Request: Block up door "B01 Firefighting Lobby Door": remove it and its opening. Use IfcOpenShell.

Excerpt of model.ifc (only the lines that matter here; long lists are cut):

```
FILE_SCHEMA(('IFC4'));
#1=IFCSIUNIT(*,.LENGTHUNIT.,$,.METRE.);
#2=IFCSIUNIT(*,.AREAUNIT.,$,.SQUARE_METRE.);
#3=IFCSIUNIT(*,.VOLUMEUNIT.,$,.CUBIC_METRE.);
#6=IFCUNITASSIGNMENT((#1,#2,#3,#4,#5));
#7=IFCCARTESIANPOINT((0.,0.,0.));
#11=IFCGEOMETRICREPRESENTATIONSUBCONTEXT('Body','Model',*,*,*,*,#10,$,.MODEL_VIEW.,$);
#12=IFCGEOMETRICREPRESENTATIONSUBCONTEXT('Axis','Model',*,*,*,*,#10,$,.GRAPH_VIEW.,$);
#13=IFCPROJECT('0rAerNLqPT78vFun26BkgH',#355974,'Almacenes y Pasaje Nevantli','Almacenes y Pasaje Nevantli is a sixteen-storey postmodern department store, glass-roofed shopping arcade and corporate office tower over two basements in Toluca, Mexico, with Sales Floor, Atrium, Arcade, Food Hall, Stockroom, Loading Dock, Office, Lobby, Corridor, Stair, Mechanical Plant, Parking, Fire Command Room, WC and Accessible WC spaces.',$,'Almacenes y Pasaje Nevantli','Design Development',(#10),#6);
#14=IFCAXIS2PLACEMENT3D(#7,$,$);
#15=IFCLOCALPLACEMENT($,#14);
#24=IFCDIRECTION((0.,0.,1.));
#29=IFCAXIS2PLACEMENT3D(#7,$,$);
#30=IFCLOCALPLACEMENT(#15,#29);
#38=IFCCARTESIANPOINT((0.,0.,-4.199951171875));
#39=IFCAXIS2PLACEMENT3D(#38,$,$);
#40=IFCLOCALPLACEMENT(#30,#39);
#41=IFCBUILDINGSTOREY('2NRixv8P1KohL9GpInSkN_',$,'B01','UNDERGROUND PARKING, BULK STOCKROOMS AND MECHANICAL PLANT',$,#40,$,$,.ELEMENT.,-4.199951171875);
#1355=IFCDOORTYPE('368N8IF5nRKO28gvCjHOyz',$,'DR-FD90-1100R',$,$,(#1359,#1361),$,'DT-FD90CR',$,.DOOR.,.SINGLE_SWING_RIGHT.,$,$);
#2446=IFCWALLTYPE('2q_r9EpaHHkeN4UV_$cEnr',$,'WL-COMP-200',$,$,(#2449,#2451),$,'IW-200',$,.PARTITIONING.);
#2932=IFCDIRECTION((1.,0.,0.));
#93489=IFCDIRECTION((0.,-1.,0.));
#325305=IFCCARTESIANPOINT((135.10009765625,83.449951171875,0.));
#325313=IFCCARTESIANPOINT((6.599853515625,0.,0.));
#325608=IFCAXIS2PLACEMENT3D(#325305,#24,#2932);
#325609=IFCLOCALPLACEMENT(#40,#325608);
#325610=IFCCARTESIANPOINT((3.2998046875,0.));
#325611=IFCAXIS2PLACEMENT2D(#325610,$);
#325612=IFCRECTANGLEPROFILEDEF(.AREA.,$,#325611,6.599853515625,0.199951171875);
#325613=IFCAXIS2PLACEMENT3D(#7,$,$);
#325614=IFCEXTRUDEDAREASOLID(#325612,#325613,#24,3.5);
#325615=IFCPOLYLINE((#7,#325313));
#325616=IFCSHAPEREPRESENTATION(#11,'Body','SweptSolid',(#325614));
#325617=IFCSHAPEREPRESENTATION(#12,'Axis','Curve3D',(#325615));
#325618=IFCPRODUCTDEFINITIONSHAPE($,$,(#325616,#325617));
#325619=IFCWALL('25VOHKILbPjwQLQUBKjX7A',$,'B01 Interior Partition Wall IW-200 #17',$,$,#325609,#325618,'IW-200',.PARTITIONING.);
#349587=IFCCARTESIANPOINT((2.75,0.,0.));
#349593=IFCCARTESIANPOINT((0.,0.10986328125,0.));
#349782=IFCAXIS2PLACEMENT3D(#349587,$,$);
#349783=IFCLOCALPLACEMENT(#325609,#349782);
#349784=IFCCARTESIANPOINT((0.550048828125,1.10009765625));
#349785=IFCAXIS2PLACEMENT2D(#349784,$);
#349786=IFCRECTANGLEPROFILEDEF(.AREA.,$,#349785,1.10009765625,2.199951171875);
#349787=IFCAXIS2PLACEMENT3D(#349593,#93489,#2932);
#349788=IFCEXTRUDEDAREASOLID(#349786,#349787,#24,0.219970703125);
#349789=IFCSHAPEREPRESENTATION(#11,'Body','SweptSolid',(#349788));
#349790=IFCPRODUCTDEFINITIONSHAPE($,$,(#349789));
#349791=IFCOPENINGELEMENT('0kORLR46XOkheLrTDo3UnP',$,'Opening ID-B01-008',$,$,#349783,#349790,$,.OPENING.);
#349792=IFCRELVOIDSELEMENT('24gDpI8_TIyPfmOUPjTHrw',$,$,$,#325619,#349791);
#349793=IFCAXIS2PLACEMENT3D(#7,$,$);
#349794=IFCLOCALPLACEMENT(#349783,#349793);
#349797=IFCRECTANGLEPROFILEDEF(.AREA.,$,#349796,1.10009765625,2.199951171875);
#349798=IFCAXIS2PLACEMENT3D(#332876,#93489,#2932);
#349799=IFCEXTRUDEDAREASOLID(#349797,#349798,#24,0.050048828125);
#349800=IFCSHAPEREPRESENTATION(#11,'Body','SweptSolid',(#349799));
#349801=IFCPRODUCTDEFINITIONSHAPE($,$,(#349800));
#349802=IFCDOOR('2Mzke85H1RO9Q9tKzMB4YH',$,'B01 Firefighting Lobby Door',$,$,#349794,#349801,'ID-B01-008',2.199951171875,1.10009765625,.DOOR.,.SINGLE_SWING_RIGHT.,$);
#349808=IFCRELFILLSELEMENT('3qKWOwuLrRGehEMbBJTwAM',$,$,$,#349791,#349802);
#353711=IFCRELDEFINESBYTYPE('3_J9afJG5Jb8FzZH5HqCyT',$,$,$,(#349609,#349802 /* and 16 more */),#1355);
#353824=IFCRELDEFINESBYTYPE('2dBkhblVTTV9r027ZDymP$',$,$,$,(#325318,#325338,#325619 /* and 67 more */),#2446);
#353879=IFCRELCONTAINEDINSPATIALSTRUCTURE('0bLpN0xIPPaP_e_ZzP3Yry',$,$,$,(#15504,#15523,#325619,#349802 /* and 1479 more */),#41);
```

```python
import ifcopenshell
import ifcopenshell.api.feature
import ifcopenshell.api.root
import ifcopenshell.geom
import ifcopenshell.util.shape

model = ifcopenshell.open("model.ifc")
settings = ifcopenshell.geom.settings()


def volume(element):
    """Net volume in cubic metres, openings subtracted."""
    shape = ifcopenshell.geom.create_shape(settings, element)
    return ifcopenshell.util.shape.get_volume(shape.geometry)


door = model.by_id(349802)
opening = door.FillsVoids[0].RelatingOpeningElement
wall = opening.VoidsElements[0].RelatingBuildingElement
before = volume(wall)

ifcopenshell.api.root.remove_product(model, product=door)
ifcopenshell.api.feature.remove_feature(model, feature=opening)

after = volume(wall)

print(f"wall volume {before:.3f} -> {after:.3f} m3")

model.write("model-out.ifc")
```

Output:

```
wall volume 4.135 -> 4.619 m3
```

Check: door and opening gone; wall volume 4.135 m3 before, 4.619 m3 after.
